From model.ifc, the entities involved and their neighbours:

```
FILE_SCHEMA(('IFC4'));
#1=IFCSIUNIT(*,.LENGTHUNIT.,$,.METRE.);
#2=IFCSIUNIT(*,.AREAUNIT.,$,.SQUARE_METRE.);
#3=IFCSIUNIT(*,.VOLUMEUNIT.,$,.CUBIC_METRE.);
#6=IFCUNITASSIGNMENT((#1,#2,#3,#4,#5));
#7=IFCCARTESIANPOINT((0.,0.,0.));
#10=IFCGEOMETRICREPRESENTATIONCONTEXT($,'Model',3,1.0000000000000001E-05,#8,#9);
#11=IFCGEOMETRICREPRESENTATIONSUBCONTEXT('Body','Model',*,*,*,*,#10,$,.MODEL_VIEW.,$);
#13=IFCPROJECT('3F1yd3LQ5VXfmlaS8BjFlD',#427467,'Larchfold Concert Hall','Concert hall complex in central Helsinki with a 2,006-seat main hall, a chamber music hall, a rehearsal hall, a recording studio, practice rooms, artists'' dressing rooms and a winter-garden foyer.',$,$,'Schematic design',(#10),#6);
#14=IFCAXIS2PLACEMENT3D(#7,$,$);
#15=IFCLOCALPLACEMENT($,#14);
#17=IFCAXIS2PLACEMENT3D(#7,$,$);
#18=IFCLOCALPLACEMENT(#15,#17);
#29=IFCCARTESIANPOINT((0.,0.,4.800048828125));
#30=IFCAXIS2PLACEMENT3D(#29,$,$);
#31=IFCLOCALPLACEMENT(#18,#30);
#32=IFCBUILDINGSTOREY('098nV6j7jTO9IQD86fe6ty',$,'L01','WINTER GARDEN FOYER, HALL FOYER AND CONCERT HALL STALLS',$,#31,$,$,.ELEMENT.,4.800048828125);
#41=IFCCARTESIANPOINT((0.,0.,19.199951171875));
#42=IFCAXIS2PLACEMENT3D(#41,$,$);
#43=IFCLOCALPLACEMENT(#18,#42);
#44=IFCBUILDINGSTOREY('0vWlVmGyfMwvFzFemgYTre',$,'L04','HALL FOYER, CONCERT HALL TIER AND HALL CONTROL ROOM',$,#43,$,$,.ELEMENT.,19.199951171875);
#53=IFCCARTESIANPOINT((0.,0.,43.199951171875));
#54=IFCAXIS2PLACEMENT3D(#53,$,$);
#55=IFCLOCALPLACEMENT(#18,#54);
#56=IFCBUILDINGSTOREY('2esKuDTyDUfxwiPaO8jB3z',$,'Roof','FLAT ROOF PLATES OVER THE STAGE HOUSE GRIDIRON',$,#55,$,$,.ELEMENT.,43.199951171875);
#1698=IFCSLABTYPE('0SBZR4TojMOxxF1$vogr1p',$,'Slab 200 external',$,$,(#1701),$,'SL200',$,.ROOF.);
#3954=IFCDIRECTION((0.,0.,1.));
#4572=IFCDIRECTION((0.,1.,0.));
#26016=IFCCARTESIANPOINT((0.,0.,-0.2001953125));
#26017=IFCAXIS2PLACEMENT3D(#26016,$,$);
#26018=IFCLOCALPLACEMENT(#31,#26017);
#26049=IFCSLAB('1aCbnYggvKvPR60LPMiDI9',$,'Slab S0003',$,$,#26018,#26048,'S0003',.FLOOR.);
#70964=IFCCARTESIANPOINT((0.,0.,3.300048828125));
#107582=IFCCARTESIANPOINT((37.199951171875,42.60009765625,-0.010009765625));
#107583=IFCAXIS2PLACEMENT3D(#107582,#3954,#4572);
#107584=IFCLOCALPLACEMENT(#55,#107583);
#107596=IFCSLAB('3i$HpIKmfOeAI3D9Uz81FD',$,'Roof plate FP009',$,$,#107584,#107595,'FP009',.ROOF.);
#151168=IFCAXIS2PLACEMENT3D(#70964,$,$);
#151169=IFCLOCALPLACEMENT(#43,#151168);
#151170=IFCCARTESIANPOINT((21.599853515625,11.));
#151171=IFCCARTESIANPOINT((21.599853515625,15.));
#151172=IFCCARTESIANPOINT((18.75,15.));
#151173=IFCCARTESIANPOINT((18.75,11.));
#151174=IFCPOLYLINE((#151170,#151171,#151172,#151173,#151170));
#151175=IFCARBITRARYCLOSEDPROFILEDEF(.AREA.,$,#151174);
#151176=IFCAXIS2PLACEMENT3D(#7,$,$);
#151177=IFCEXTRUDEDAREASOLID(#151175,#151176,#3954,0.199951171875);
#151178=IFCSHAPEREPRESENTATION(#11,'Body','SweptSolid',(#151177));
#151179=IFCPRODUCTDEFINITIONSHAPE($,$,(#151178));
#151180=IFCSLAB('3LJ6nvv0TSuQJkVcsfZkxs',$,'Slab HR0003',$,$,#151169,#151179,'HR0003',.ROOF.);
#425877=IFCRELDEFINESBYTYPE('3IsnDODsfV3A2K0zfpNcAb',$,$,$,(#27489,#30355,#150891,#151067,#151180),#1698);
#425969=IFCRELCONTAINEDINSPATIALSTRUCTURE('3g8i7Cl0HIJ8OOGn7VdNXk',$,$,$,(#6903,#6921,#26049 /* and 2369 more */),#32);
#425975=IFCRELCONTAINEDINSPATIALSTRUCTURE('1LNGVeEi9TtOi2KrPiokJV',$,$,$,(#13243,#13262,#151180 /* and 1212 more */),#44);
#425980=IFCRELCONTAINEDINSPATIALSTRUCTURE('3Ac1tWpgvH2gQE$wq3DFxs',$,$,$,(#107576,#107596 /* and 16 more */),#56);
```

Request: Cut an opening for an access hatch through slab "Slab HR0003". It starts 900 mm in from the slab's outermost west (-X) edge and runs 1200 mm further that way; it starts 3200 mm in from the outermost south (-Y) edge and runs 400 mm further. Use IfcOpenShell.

```python
import numpy as np
import ifcopenshell
import ifcopenshell.api.feature
import ifcopenshell.api.geometry
import ifcopenshell.api.root
import ifcopenshell.geom
import ifcopenshell.util.placement
import ifcopenshell.util.representation
import ifcopenshell.util.shape
import ifcopenshell.util.unit

model = ifcopenshell.open("model.ifc")
unit_scale = ifcopenshell.util.unit.calculate_unit_scale(model)
settings = ifcopenshell.geom.settings()


def volume(element):
    """Net volume in cubic metres, openings subtracted."""
    shape = ifcopenshell.geom.create_shape(settings, element)
    return ifcopenshell.util.shape.get_volume(shape.geometry)


slab = model.by_guid("3LJ6nvv0TSuQJkVcsfZkxs")
before = volume(slab)

# Extent in the slab's own axes, in metres. The edges named are its -X and -Y sides.
slab_shape = ifcopenshell.geom.create_shape(settings, slab)
vertices = ifcopenshell.util.shape.get_vertices(slab_shape.geometry)
x_min, y_min, bottom = vertices.min(axis=0)
top = vertices[:, 2].max()

opening = ifcopenshell.api.root.create_entity(model, ifc_class="IfcOpeningElement", name="Access hatch opening", predefined_type="OPENING")
context = ifcopenshell.util.representation.get_context(model, "Model", "Body", "MODEL_VIEW")
width, depth = 1.2, 0.4
outline = [(0.0, 0.0), (width, 0.0), (width, depth), (0.0, depth), (0.0, 0.0)]
# Overshoot both faces by 50 mm so the cut is clean.
shape = ifcopenshell.api.geometry.add_slab_representation(
    model, context=context, depth=top - bottom + 0.1, polyline=outline
)
ifcopenshell.api.geometry.assign_representation(model, product=opening, representation=shape)

matrix = ifcopenshell.util.placement.get_local_placement(slab.ObjectPlacement)
matrix[:, 3] = matrix @ np.append(np.array([x_min + 0.9, y_min + 3.2, bottom - 0.05]) / unit_scale, 1.0)
ifcopenshell.api.geometry.edit_object_placement(model, product=opening, matrix=matrix, is_si=False)
ifcopenshell.api.feature.add_feature(model, feature=opening, element=slab)

after = volume(slab)

print(f"slab volume {before:.3f} -> {after:.3f} m3")

model.write("model_updated.ifc")
```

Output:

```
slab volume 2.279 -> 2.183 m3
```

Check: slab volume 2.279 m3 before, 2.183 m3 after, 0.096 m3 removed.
